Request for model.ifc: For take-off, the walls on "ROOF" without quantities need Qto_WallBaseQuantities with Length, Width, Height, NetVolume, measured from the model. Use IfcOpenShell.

First a look at what the model holds.

```python
import ifcopenshell
import ifcopenshell.util.element
import ifcopenshell.util.unit

model = ifcopenshell.open("model.ifc")
print(model.schema)
for unit_type in ("LENGTHUNIT", "AREAUNIT", "VOLUMEUNIT"):
    print(unit_type, ifcopenshell.util.unit.calculate_unit_scale(model, unit_type))
storey = next(s for s in model.by_type("IfcBuildingStorey") if s.Name == "ROOF")
walls = [e for e in ifcopenshell.util.element.get_decomposition(storey) if e.is_a("IfcWall")]
for e in sorted(walls, key=lambda e: e.id()):
    print(e.id(), e.is_a(), e.Name, list(ifcopenshell.util.element.get_psets(e, qtos_only=True)), sep=" | ")
```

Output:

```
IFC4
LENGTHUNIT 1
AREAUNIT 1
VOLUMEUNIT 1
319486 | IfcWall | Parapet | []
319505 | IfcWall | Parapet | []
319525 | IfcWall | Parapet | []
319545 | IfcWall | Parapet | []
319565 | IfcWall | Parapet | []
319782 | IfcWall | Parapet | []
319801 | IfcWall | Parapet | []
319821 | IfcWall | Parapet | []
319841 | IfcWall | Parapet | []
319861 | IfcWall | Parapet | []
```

```python
import ifcopenshell
import ifcopenshell.api.pset
import ifcopenshell.geom
import ifcopenshell.util.element
import ifcopenshell.util.shape
import ifcopenshell.util.unit

model = ifcopenshell.open("model.ifc")
unit_scale = ifcopenshell.util.unit.calculate_unit_scale(model)
volume_scale = ifcopenshell.util.unit.calculate_unit_scale(model, "VOLUMEUNIT")
settings = ifcopenshell.geom.settings()

storey = next(s for s in model.by_type("IfcBuildingStorey") if s.Name == "ROOF")
walls = [e for e in ifcopenshell.util.element.get_decomposition(storey) if e.is_a("IfcWall")]

for e in sorted(walls, key=lambda e: e.id()):
    if ifcopenshell.util.element.get_psets(e, qtos_only=True, should_inherit=False):
        continue
    # Geometry comes back in metres, in the element's own axes.
    shape = ifcopenshell.geom.create_shape(settings, e)
    values = {
        "Length": ifcopenshell.util.shape.get_x(shape.geometry) / unit_scale,
        "Width": ifcopenshell.util.shape.get_y(shape.geometry) / unit_scale,
        "Height": ifcopenshell.util.shape.get_z(shape.geometry) / unit_scale,
        "NetVolume": ifcopenshell.util.shape.get_volume(shape.geometry) / volume_scale,
    }
    qto = ifcopenshell.api.pset.add_qto(model, product=e, name="Qto_WallBaseQuantities")
    ifcopenshell.api.pset.edit_qto(model, qto=qto, properties=values)
    print(e.id(), {k: round(v, 3) for k, v in values.items()})

model.write("model_updated.ifc")
```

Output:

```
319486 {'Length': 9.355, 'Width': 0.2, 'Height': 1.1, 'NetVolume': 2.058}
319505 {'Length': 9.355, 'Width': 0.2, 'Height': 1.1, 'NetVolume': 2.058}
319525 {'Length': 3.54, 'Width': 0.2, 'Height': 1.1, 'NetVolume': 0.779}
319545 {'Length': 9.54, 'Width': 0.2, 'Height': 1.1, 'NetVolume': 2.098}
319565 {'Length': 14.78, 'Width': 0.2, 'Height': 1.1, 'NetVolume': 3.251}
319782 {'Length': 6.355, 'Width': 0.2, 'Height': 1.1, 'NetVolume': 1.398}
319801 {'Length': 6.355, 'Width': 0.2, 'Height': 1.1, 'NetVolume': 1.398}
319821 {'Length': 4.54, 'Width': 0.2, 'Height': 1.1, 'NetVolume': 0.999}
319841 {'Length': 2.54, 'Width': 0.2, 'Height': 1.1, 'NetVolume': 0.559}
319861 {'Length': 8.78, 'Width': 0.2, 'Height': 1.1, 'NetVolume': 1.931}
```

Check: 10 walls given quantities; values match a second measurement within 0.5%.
